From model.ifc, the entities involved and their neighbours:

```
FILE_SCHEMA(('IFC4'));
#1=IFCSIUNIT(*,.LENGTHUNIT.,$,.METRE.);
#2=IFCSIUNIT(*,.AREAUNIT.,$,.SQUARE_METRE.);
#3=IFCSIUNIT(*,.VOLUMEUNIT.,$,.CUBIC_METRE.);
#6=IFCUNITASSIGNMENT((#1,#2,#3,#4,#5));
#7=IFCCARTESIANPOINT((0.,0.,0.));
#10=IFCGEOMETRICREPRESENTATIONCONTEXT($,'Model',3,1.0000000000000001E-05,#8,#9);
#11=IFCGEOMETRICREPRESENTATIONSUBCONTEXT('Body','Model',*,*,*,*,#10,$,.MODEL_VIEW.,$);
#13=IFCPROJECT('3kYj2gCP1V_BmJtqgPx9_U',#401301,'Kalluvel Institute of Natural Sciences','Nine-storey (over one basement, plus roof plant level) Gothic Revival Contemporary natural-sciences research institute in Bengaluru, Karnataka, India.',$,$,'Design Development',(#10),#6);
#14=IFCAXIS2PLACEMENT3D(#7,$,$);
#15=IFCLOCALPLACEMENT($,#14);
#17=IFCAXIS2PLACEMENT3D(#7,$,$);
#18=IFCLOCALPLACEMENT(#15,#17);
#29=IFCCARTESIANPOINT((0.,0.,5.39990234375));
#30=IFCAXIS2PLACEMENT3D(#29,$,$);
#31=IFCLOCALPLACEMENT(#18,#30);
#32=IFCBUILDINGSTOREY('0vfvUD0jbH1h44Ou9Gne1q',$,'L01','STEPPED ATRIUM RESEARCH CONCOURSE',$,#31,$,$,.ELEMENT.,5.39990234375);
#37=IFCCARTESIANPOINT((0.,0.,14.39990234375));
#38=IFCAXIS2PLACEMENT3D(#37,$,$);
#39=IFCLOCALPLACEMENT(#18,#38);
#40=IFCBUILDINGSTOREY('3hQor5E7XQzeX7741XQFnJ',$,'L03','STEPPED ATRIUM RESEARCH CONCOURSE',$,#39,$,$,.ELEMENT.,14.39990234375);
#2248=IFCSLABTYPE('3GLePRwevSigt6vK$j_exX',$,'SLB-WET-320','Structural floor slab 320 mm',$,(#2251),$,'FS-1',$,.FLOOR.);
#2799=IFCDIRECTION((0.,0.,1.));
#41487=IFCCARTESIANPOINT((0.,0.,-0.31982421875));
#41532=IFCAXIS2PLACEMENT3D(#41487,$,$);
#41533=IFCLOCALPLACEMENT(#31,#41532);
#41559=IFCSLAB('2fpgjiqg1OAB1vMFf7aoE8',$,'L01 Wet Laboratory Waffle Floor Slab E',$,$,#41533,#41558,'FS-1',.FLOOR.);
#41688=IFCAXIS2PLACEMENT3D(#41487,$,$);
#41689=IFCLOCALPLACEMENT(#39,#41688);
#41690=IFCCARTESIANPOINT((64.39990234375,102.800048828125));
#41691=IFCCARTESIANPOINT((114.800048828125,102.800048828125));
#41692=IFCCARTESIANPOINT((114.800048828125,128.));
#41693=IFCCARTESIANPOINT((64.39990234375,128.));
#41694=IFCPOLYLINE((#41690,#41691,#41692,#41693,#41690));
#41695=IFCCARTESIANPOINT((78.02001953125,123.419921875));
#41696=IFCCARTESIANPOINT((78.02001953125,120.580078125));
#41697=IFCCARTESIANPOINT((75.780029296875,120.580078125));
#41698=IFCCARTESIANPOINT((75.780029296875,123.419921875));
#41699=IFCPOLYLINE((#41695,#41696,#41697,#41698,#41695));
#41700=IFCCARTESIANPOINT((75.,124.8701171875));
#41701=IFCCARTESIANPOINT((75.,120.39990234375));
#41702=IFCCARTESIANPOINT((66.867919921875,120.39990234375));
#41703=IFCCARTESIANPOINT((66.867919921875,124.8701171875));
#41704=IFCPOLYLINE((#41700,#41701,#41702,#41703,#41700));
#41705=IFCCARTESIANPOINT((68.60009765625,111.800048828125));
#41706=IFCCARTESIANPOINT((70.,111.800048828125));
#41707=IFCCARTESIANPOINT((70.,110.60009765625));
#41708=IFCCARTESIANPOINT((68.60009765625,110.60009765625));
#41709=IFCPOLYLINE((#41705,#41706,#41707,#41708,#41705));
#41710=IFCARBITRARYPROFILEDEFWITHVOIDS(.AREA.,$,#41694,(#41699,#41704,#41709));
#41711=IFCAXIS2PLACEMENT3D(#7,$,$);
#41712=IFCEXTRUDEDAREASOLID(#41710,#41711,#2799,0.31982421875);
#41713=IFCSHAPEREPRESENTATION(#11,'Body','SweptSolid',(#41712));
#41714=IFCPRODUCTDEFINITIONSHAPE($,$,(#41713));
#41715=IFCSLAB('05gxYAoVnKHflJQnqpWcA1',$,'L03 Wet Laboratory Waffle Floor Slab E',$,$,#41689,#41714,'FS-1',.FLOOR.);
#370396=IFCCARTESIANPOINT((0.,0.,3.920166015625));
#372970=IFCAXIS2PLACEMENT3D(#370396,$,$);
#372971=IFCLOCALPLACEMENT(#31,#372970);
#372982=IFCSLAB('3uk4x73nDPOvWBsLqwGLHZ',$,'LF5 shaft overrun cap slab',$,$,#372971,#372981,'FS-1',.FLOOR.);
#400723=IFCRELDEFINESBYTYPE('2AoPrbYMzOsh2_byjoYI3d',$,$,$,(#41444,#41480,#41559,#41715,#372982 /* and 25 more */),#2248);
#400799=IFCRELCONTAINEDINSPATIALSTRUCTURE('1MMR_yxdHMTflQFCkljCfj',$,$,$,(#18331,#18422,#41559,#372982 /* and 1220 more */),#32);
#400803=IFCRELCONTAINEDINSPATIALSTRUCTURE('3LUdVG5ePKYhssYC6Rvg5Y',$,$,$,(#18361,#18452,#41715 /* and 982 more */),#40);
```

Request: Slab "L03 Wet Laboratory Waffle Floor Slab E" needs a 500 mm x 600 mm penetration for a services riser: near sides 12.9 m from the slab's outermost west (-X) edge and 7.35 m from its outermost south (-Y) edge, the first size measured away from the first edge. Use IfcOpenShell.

```python
import numpy as np
import ifcopenshell
import ifcopenshell.api.feature
import ifcopenshell.api.geometry
import ifcopenshell.api.root
import ifcopenshell.geom
import ifcopenshell.util.placement
import ifcopenshell.util.representation
import ifcopenshell.util.shape
import ifcopenshell.util.unit

model = ifcopenshell.open("model.ifc")
unit_scale = ifcopenshell.util.unit.calculate_unit_scale(model)
settings = ifcopenshell.geom.settings()


def volume(element):
    """Net volume in cubic metres, openings subtracted."""
    shape = ifcopenshell.geom.create_shape(settings, element)
    return ifcopenshell.util.shape.get_volume(shape.geometry)


slab = model.by_guid("05gxYAoVnKHflJQnqpWcA1")
before = volume(slab)

# Extent in the slab's own axes, in metres. The edges named are its -X and -Y sides.
slab_shape = ifcopenshell.geom.create_shape(settings, slab)
vertices = ifcopenshell.util.shape.get_vertices(slab_shape.geometry)
x_min, y_min, bottom = vertices.min(axis=0)
top = vertices[:, 2].max()

opening = ifcopenshell.api.root.create_entity(model, ifc_class="IfcOpeningElement", name="Services riser opening", predefined_type="OPENING")
context = ifcopenshell.util.representation.get_context(model, "Model", "Body", "MODEL_VIEW")
width, depth = 0.5, 0.6
outline = [(0.0, 0.0), (width, 0.0), (width, depth), (0.0, depth), (0.0, 0.0)]
# Overshoot both faces by 50 mm so the cut is clean.
shape = ifcopenshell.api.geometry.add_slab_representation(
    model, context=context, depth=top - bottom + 0.1, polyline=outline
)
ifcopenshell.api.geometry.assign_representation(model, product=opening, representation=shape)

matrix = ifcopenshell.util.placement.get_local_placement(slab.ObjectPlacement)
matrix[:, 3] = matrix @ np.append(np.array([x_min + 12.9, y_min + 7.35, bottom - 0.05]) / unit_scale, 1.0)
ifcopenshell.api.geometry.edit_object_placement(model, product=opening, matrix=matrix, is_si=False)
ifcopenshell.api.feature.add_feature(model, feature=opening, element=slab)

after = volume(slab)

print(f"slab volume {before:.3f} -> {after:.3f} m3")

model.write("model_updated.ifc")
```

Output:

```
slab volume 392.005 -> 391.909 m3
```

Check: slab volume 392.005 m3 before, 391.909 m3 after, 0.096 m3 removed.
